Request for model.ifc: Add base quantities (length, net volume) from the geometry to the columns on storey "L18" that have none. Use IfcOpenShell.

First a look at what the model holds.

```python
import ifcopenshell
import ifcopenshell.util.element
import ifcopenshell.util.unit

model = ifcopenshell.open("model.ifc")
print(model.schema)
for unit_type in ("LENGTHUNIT", "AREAUNIT", "VOLUMEUNIT"):
    print(unit_type, ifcopenshell.util.unit.calculate_unit_scale(model, unit_type))
storey = next(s for s in model.by_type("IfcBuildingStorey") if s.Name == "L18")
columns = [e for e in ifcopenshell.util.element.get_decomposition(storey) if e.is_a("IfcColumn")]
for e in sorted(columns, key=lambda e: e.id()):
    print(e.id(), e.is_a(), e.Name, list(ifcopenshell.util.element.get_psets(e, qtos_only=True)), sep=" | ")
```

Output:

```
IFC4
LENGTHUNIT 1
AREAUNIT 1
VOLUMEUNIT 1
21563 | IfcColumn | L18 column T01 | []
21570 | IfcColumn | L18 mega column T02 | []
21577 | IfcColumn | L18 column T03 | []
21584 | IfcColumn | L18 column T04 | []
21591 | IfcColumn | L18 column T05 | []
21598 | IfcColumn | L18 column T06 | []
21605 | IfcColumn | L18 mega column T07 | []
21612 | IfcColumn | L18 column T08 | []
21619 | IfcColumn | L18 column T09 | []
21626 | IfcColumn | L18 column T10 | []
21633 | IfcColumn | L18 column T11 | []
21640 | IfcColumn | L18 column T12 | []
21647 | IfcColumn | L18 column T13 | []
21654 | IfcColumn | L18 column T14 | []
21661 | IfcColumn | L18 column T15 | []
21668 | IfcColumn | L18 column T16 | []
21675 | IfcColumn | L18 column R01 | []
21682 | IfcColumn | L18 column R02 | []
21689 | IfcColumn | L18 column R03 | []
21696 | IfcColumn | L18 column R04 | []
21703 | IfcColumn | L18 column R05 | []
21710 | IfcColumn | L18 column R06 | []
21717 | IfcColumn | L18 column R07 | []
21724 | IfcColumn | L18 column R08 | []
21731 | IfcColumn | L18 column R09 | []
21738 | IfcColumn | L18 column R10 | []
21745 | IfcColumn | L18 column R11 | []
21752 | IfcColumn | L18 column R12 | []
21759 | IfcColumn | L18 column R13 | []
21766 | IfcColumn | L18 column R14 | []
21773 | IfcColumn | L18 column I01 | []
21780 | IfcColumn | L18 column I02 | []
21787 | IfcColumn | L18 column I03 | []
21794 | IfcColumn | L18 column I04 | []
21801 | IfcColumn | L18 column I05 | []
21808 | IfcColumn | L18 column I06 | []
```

```python
import ifcopenshell
import ifcopenshell.api.pset
import ifcopenshell.geom
import ifcopenshell.util.element
import ifcopenshell.util.shape
import ifcopenshell.util.unit

model = ifcopenshell.open("model.ifc")
unit_scale = ifcopenshell.util.unit.calculate_unit_scale(model)
volume_scale = ifcopenshell.util.unit.calculate_unit_scale(model, "VOLUMEUNIT")
settings = ifcopenshell.geom.settings()

storey = next(s for s in model.by_type("IfcBuildingStorey") if s.Name == "L18")
columns = [e for e in ifcopenshell.util.element.get_decomposition(storey) if e.is_a("IfcColumn")]

for e in sorted(columns, key=lambda e: e.id()):
    if ifcopenshell.util.element.get_psets(e, qtos_only=True, should_inherit=False):
        continue
    # Geometry comes back in metres, in the element's own axes.
    shape = ifcopenshell.geom.create_shape(settings, e)
    values = {
        "Length": ifcopenshell.util.shape.get_z(shape.geometry) / unit_scale,
        "NetVolume": ifcopenshell.util.shape.get_volume(shape.geometry) / volume_scale,
    }
    qto = ifcopenshell.api.pset.add_qto(model, product=e, name="Qto_ColumnBaseQuantities")
    ifcopenshell.api.pset.edit_qto(model, qto=qto, properties=values)
    print(e.id(), {k: round(v, 3) for k, v in values.items()})

model.write("model_edited.ifc")
```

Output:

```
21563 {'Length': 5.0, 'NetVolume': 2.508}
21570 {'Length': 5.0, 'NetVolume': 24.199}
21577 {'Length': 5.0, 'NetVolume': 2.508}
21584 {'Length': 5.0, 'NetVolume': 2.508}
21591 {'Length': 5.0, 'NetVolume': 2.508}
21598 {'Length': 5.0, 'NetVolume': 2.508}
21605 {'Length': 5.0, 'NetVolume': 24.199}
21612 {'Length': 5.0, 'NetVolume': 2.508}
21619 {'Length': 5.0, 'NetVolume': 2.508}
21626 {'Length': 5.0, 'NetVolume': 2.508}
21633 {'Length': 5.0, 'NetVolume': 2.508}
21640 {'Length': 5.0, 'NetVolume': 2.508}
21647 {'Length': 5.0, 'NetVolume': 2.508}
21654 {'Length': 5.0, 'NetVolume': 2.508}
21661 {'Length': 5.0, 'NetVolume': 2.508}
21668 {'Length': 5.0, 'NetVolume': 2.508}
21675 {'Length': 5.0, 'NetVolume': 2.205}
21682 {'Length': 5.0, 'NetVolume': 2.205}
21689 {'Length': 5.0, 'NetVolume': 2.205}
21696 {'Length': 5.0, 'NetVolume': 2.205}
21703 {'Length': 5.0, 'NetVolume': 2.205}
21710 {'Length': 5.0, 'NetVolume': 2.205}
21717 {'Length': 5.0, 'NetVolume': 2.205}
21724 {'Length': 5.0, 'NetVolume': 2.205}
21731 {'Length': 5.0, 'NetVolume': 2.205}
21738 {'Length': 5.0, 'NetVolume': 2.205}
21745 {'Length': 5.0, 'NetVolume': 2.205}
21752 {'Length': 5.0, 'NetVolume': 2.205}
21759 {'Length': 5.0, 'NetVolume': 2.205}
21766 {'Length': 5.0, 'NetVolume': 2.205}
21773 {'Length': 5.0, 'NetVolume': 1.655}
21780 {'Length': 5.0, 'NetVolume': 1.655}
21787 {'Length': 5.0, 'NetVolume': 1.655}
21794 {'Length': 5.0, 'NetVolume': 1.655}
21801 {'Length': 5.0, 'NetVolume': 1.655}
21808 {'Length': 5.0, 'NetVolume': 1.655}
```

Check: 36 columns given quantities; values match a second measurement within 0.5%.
